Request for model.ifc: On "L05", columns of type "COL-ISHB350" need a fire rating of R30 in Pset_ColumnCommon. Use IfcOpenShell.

First a look at what the model holds.

```python
import ifcopenshell
import ifcopenshell.util.element

model = ifcopenshell.open("model.ifc")
print(model.schema)
storey = next(s for s in model.by_type("IfcBuildingStorey") if s.Name == "L05")
columns = [e for e in ifcopenshell.util.element.get_decomposition(storey) if e.is_a("IfcColumn")]
seen = {}
for e in columns:
    element_type = ifcopenshell.util.element.get_type(e)
    key = (element_type.Name if element_type != e and element_type else None, ifcopenshell.util.element.get_pset(e, "Pset_ColumnCommon", "FireRating"))
    seen[key] = seen.get(key, 0) + 1
for (name, value), count in sorted(seen.items(), key=str):
    print(count, "x", name, "|", value)
```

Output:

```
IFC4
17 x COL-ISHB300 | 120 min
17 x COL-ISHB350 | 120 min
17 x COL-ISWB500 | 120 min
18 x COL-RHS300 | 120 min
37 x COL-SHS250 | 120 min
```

```python
import ifcopenshell
import ifcopenshell.api.pset
import ifcopenshell.util.element

model = ifcopenshell.open("model.ifc")

storey = next(s for s in model.by_type("IfcBuildingStorey") if s.Name == "L05")
columns = [e for e in ifcopenshell.util.element.get_decomposition(storey) if e.is_a("IfcColumn")]

count = 0
for e in columns:
    element_type = ifcopenshell.util.element.get_type(e)
    if element_type in (None, e) or element_type.Name != "COL-ISHB350":
        continue
    # add_pset returns the element's existing set when there is one.
    pset = ifcopenshell.api.pset.add_pset(model, product=e, name="Pset_ColumnCommon")
    ifcopenshell.api.pset.edit_pset(model, pset=pset, properties={"FireRating": "R30"})
    count += 1

print(count, "columns updated")

model.write("model_v2.ifc")
```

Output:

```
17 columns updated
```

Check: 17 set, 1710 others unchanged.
